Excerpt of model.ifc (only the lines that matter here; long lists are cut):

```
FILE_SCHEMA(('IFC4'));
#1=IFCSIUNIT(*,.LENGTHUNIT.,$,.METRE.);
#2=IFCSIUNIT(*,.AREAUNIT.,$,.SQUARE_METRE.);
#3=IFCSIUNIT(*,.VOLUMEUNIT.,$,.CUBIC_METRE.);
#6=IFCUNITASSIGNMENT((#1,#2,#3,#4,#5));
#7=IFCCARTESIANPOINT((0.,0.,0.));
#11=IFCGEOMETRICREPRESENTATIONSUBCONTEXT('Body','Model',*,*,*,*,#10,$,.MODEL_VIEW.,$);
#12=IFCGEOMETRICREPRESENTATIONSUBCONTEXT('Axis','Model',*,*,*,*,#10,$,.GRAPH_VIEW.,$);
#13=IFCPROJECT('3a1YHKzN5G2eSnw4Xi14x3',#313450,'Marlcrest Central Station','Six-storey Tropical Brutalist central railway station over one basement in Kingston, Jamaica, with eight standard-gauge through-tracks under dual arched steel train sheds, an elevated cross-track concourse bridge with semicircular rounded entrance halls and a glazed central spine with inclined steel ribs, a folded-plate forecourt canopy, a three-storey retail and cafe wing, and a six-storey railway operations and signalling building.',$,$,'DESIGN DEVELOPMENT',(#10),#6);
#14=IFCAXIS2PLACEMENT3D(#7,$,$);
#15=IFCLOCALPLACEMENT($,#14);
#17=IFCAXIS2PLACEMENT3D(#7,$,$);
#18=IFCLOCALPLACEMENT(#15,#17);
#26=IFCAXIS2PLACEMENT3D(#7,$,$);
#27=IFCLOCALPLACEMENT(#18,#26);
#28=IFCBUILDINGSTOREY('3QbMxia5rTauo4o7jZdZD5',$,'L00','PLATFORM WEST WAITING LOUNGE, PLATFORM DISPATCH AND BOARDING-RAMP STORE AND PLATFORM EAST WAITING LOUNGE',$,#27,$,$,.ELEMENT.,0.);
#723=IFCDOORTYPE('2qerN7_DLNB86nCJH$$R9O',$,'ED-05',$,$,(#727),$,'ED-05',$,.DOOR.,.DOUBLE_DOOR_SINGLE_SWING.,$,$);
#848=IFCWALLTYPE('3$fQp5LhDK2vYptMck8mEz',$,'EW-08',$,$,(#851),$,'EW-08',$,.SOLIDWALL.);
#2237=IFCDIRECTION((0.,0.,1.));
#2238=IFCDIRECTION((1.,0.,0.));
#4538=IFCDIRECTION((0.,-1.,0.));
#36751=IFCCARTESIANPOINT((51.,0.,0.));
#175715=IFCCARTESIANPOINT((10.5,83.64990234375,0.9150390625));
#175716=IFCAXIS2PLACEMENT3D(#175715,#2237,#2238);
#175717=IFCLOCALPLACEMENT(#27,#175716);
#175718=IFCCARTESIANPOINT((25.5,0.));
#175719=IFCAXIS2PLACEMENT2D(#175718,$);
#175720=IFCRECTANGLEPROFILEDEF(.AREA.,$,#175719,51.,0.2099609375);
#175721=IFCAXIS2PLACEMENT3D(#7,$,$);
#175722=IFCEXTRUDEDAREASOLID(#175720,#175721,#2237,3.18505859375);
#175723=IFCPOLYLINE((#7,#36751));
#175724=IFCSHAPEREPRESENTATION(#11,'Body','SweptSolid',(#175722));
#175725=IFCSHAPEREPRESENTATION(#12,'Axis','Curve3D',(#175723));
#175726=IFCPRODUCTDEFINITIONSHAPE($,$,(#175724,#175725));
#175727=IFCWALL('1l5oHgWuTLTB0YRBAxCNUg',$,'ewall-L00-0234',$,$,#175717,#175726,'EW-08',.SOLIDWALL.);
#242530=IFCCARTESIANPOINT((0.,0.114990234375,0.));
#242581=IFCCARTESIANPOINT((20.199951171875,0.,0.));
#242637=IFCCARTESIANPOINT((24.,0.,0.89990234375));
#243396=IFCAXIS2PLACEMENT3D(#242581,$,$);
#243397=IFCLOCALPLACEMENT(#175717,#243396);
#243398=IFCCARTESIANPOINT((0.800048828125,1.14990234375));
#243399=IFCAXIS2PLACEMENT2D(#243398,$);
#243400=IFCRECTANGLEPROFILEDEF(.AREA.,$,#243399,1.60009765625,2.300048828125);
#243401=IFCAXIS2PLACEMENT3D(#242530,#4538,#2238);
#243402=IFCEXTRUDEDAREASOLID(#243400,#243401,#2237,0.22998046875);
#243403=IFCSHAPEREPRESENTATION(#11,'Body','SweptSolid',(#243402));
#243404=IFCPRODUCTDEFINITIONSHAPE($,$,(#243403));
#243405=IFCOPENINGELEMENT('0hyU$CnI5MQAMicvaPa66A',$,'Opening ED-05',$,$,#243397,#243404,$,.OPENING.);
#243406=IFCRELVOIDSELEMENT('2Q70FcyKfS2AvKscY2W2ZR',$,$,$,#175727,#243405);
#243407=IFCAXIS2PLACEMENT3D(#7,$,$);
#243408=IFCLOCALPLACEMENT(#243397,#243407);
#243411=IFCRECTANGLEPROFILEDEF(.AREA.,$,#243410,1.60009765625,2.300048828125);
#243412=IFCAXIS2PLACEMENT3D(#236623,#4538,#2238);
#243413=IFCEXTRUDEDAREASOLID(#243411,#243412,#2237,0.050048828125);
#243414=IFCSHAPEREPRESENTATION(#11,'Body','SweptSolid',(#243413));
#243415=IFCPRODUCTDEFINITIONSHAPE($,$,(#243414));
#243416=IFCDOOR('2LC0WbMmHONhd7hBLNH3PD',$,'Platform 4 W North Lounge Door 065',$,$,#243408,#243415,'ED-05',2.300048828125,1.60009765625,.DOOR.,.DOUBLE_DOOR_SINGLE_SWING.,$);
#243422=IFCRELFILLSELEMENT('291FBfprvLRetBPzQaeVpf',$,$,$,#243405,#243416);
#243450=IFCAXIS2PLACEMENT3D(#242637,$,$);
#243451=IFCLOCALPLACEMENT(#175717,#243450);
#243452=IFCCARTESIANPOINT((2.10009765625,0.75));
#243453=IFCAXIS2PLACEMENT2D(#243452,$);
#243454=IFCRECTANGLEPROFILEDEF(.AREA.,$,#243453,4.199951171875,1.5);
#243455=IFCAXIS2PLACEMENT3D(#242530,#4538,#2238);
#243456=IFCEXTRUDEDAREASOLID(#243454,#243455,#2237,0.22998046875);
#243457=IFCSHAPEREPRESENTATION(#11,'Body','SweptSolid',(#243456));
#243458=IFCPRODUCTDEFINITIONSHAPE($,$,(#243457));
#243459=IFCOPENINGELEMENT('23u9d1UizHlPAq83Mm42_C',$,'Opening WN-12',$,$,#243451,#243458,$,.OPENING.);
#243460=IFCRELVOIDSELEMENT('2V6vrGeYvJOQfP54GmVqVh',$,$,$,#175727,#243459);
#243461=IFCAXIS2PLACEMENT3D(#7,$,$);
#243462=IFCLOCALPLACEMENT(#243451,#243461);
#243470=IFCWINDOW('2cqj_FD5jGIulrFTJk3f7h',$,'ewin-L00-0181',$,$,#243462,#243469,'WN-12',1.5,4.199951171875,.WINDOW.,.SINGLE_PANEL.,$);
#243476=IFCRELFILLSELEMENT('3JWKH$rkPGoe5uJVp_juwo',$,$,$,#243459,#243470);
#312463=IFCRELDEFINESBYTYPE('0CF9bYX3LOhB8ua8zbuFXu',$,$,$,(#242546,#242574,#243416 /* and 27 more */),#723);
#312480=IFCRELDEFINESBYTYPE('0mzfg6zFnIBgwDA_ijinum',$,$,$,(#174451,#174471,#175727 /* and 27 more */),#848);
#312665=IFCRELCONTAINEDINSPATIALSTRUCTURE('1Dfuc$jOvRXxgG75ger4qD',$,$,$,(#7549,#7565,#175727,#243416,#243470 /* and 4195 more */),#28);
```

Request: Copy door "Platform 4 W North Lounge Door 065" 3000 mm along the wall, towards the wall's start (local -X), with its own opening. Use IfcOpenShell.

```python
import ifcopenshell
import ifcopenshell.api.feature
import ifcopenshell.api.geometry
import ifcopenshell.api.root
import ifcopenshell.geom
import ifcopenshell.util.element
import ifcopenshell.util.placement
import ifcopenshell.util.shape
import ifcopenshell.util.unit

model = ifcopenshell.open("model.ifc")
unit_scale = ifcopenshell.util.unit.calculate_unit_scale(model)
settings = ifcopenshell.geom.settings()


def volume(element):
    """Net volume in cubic metres, openings subtracted."""
    shape = ifcopenshell.geom.create_shape(settings, element)
    return ifcopenshell.util.shape.get_volume(shape.geometry)


door = model.by_id(243416)
opening = door.FillsVoids[0].RelatingOpeningElement
wall = opening.VoidsElements[0].RelatingBuildingElement
before = volume(wall)
shift = ifcopenshell.util.placement.get_local_placement(wall.ObjectPlacement)[:3, 0] * -3 / unit_scale

# copy_class copies the void relationship, type, container and properties, but no geometry.
new_opening = ifcopenshell.api.root.copy_class(model, product=opening)
new_opening.Representation = ifcopenshell.util.element.copy_deep(
    model, opening.Representation, exclude=["IfcGeometricRepresentationContext", "IfcRepresentationMap"]
)
new_door = ifcopenshell.api.root.copy_class(model, product=door)
new_door.Representation = ifcopenshell.util.element.copy_deep(
    model, door.Representation, exclude=["IfcGeometricRepresentationContext", "IfcRepresentationMap"]
)
new_door.Tag = None
ifcopenshell.api.feature.add_filling(model, opening=new_opening, element=new_door)

for old, new in ((opening, new_opening), (door, new_door)):
    matrix = ifcopenshell.util.placement.get_local_placement(old.ObjectPlacement)
    matrix[:3, 3] += shift
    ifcopenshell.api.geometry.edit_object_placement(model, product=new, matrix=matrix, is_si=False)

after = volume(wall)

print(f"wall volume {before:.3f} -> {after:.3f} m3")

model.write("model_rev.ifc")
```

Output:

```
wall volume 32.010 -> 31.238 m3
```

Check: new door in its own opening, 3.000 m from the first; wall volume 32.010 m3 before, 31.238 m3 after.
